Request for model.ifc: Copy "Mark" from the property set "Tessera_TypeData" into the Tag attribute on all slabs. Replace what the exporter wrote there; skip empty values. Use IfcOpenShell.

First a look at what the model holds.

```python
import ifcopenshell
import ifcopenshell.util.element

model = ifcopenshell.open("model.ifc")
print(model.schema)
slabs = model.by_type("IfcSlab")
print(len(slabs), "slabs")
for e in slabs[:8]:
    source = ifcopenshell.util.element.get_pset(e, "Tessera_TypeData", "Mark")
    target = e.Tag
    print(e.id(), repr(source), repr(target), sep=" | ")
```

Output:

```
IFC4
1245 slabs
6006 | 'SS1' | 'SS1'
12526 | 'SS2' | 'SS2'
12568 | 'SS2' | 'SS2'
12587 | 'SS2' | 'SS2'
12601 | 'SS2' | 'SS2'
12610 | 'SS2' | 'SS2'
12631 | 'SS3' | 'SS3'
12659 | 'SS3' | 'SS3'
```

```python
import ifcopenshell
import ifcopenshell.util.element

model = ifcopenshell.open("model.ifc")

count = 0
for e in model.by_type("IfcSlab"):
    value = ifcopenshell.util.element.get_pset(e, "Tessera_TypeData", "Mark")
    current = e.Tag
    if not value or not value.strip() or current == value:
        continue
    e.Tag = value
    count += 1

print(count, "slabs updated")

model.write("model_rev.ifc")
```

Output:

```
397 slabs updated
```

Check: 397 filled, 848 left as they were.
